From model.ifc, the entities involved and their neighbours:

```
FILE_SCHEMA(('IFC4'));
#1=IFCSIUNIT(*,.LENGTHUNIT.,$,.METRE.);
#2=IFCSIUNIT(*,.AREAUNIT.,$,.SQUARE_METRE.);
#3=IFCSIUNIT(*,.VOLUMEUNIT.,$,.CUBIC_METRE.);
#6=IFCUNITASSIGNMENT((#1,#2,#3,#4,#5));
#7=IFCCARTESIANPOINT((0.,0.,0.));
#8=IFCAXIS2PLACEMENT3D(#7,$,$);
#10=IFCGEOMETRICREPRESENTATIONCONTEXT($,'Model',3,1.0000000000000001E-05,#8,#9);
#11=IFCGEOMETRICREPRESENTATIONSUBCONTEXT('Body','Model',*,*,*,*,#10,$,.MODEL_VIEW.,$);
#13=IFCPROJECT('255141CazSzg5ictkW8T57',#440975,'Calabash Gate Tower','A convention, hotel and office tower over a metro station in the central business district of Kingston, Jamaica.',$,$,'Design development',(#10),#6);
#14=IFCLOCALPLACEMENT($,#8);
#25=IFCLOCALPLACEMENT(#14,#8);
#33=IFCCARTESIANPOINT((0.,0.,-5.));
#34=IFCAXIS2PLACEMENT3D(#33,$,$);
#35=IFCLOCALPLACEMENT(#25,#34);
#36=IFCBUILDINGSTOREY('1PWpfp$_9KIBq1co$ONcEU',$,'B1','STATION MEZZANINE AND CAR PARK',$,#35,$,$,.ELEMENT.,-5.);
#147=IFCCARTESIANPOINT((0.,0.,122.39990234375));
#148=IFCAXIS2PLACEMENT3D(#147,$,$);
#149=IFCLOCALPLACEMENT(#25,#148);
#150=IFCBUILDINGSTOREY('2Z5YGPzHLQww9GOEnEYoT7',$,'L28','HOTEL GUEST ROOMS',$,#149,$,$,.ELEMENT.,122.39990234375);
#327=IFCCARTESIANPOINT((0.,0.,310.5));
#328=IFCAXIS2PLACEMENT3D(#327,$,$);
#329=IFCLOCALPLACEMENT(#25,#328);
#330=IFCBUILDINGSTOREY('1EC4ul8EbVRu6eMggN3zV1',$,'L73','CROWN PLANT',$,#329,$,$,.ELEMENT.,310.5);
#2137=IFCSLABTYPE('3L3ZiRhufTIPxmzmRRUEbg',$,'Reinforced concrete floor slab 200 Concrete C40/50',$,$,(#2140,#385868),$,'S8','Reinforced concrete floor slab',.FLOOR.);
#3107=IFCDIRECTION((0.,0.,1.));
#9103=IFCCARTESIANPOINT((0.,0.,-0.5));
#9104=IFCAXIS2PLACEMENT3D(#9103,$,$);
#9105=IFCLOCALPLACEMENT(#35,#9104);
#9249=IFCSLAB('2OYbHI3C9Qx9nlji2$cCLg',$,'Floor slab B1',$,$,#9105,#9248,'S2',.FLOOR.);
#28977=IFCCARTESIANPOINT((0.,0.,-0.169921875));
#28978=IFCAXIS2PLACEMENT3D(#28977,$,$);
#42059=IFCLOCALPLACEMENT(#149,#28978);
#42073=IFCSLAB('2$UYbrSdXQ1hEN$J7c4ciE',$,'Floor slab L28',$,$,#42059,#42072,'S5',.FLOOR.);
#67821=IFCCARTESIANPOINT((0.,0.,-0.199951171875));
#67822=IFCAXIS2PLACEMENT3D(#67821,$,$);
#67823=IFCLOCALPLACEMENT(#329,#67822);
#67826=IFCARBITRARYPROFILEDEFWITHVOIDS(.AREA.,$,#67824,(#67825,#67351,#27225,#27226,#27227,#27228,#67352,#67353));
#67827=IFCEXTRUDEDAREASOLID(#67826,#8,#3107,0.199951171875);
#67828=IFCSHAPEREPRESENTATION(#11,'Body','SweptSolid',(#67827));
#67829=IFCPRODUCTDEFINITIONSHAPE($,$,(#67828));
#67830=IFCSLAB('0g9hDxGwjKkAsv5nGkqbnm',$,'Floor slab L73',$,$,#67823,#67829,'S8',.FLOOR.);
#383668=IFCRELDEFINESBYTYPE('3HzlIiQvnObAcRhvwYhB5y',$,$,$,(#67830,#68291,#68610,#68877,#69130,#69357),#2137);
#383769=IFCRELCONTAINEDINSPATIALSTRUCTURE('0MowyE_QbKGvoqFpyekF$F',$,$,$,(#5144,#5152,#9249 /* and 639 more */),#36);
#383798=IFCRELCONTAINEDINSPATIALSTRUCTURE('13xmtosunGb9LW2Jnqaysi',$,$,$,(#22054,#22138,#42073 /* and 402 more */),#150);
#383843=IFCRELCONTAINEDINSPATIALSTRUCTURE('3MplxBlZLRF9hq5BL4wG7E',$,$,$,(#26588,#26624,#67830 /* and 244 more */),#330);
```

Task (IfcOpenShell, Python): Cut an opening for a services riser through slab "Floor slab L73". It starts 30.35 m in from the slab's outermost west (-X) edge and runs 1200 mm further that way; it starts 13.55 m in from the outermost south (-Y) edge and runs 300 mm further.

```python
import numpy as np
import ifcopenshell
import ifcopenshell.api.feature
import ifcopenshell.api.geometry
import ifcopenshell.api.root
import ifcopenshell.geom
import ifcopenshell.util.placement
import ifcopenshell.util.representation
import ifcopenshell.util.shape
import ifcopenshell.util.unit

model = ifcopenshell.open("model.ifc")
unit_scale = ifcopenshell.util.unit.calculate_unit_scale(model)
settings = ifcopenshell.geom.settings()


def volume(element):
    """Net volume in cubic metres, openings subtracted."""
    shape = ifcopenshell.geom.create_shape(settings, element)
    return ifcopenshell.util.shape.get_volume(shape.geometry)


slab = model.by_id(67830)
before = volume(slab)

# Extent in the slab's own axes, in metres. The edges named are its -X and -Y sides.
slab_shape = ifcopenshell.geom.create_shape(settings, slab)
vertices = ifcopenshell.util.shape.get_vertices(slab_shape.geometry)
x_min, y_min, bottom = vertices.min(axis=0)
top = vertices[:, 2].max()

opening = ifcopenshell.api.root.create_entity(model, ifc_class="IfcOpeningElement", name="Services riser opening", predefined_type="OPENING")
context = ifcopenshell.util.representation.get_context(model, "Model", "Body", "MODEL_VIEW")
width, depth = 1.2, 0.3
outline = [(0.0, 0.0), (width, 0.0), (width, depth), (0.0, depth), (0.0, 0.0)]
# Overshoot both faces by 50 mm so the cut is clean.
shape = ifcopenshell.api.geometry.add_slab_representation(
    model, context=context, depth=top - bottom + 0.1, polyline=outline
)
ifcopenshell.api.geometry.assign_representation(model, product=opening, representation=shape)

matrix = ifcopenshell.util.placement.get_local_placement(slab.ObjectPlacement)
matrix[:, 3] = matrix @ np.append(np.array([x_min + 30.35, y_min + 13.55, bottom - 0.05]) / unit_scale, 1.0)
ifcopenshell.api.geometry.edit_object_placement(model, product=opening, matrix=matrix, is_si=False)
ifcopenshell.api.feature.add_feature(model, feature=opening, element=slab)

after = volume(slab)

print(f"slab volume {before:.3f} -> {after:.3f} m3")

model.write("model_updated.ifc")
```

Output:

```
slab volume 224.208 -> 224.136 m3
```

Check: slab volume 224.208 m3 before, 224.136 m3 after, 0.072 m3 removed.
